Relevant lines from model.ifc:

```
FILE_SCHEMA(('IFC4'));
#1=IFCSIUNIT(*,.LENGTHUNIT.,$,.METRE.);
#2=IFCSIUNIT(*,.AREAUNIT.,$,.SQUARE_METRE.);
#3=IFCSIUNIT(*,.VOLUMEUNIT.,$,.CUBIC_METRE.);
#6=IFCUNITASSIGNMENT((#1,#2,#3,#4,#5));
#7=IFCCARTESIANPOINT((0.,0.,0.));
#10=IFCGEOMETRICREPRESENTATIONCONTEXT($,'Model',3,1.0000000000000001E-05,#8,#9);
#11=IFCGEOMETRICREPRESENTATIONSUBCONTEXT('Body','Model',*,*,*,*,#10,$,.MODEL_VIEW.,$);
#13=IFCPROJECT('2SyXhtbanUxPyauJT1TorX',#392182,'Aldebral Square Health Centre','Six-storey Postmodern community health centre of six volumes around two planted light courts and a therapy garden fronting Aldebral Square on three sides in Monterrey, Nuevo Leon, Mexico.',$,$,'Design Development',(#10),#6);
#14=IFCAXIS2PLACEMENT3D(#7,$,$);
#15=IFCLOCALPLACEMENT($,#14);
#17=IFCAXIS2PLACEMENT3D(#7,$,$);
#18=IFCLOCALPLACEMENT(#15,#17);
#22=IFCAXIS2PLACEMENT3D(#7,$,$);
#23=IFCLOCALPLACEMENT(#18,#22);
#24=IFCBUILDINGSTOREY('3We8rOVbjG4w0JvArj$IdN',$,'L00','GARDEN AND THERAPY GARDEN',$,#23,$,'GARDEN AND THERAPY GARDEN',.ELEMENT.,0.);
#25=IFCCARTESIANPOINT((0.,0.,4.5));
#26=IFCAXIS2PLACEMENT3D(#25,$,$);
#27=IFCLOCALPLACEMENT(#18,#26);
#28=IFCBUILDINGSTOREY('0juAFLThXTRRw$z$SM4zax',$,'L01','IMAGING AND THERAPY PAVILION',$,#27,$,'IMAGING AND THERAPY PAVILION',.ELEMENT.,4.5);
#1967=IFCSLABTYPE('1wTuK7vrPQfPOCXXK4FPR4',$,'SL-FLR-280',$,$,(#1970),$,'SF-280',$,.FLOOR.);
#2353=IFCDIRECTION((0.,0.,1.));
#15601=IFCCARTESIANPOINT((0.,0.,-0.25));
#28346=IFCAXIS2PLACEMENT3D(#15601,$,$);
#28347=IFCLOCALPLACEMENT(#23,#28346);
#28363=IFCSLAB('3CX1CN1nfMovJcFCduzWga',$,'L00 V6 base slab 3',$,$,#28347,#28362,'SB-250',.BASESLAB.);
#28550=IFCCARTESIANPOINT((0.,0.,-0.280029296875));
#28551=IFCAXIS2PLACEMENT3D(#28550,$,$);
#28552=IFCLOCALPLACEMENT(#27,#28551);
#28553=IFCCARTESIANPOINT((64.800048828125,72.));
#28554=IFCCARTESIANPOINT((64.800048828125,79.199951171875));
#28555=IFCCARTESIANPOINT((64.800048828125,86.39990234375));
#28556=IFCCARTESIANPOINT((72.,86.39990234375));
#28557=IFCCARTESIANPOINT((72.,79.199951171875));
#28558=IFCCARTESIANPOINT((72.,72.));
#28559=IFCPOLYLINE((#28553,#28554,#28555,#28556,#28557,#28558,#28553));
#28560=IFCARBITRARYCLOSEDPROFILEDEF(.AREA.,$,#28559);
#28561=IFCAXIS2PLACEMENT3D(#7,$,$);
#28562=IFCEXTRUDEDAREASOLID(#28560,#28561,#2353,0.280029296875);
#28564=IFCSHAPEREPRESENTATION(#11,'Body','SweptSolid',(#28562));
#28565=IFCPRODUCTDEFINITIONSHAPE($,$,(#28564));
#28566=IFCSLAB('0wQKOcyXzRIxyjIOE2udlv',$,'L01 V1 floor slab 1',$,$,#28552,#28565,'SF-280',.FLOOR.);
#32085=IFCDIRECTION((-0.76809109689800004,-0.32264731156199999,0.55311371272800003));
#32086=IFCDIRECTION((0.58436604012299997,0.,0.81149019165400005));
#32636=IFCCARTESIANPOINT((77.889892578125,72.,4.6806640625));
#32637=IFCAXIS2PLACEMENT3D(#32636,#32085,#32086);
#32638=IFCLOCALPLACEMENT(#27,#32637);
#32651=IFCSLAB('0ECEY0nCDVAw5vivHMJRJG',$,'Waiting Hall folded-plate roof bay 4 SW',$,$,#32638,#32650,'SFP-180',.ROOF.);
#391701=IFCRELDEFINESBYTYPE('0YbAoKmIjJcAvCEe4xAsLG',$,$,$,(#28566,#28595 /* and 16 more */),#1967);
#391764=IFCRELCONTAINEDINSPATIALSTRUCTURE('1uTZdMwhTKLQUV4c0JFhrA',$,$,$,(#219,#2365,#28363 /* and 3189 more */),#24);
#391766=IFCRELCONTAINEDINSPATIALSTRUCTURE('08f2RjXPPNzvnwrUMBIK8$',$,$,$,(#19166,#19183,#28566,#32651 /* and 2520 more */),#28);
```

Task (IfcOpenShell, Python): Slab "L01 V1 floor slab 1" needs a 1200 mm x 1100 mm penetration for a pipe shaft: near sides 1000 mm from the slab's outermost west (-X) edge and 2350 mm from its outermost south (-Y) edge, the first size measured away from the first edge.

```python
import numpy as np
import ifcopenshell
import ifcopenshell.api.feature
import ifcopenshell.api.geometry
import ifcopenshell.api.root
import ifcopenshell.geom
import ifcopenshell.util.placement
import ifcopenshell.util.representation
import ifcopenshell.util.shape
import ifcopenshell.util.unit

model = ifcopenshell.open("model.ifc")
unit_scale = ifcopenshell.util.unit.calculate_unit_scale(model)
settings = ifcopenshell.geom.settings()


def volume(element):
    """Net volume in cubic metres, openings subtracted."""
    shape = ifcopenshell.geom.create_shape(settings, element)
    return ifcopenshell.util.shape.get_volume(shape.geometry)


slab = model.by_guid("0wQKOcyXzRIxyjIOE2udlv")
before = volume(slab)

# Extent in the slab's own axes, in metres. The edges named are its -X and -Y sides.
slab_shape = ifcopenshell.geom.create_shape(settings, slab)
vertices = ifcopenshell.util.shape.get_vertices(slab_shape.geometry)
x_min, y_min, bottom = vertices.min(axis=0)
top = vertices[:, 2].max()

opening = ifcopenshell.api.root.create_entity(model, ifc_class="IfcOpeningElement", name="Pipe shaft opening", predefined_type="OPENING")
context = ifcopenshell.util.representation.get_context(model, "Model", "Body", "MODEL_VIEW")
width, depth = 1.2, 1.1
outline = [(0.0, 0.0), (width, 0.0), (width, depth), (0.0, depth), (0.0, 0.0)]
# Overshoot both faces by 50 mm so the cut is clean.
shape = ifcopenshell.api.geometry.add_slab_representation(
    model, context=context, depth=top - bottom + 0.1, polyline=outline
)
ifcopenshell.api.geometry.assign_representation(model, product=opening, representation=shape)

matrix = ifcopenshell.util.placement.get_local_placement(slab.ObjectPlacement)
matrix[:, 3] = matrix @ np.append(np.array([x_min + 1, y_min + 2.35, bottom - 0.05]) / unit_scale, 1.0)
ifcopenshell.api.geometry.edit_object_placement(model, product=opening, matrix=matrix, is_si=False)
ifcopenshell.api.feature.add_feature(model, feature=opening, element=slab)

after = volume(slab)

print(f"slab volume {before:.3f} -> {after:.3f} m3")

model.write("model-out.ifc")
```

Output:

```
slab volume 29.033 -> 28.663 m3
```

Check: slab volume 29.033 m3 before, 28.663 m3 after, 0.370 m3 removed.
